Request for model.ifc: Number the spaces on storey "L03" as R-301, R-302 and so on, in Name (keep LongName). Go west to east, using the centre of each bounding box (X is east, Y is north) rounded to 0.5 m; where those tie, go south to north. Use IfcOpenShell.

First a look at what the model holds.

```python
import ifcopenshell
import ifcopenshell.util.element
import ifcopenshell.util.placement

model = ifcopenshell.open("model.ifc")
print(model.schema)
storey = next(s for s in model.by_type("IfcBuildingStorey") if s.Name == "L03")
spaces = [e for e in ifcopenshell.util.element.get_decomposition(storey) if e.is_a("IfcSpace")]
for e in sorted(spaces, key=lambda e: e.id()):
    origin = ifcopenshell.util.placement.get_local_placement(e.ObjectPlacement)[:3, 3]
    print(e.id(), e.Name, e.LongName, origin.round(2) + 0.0, sep=" | ")
```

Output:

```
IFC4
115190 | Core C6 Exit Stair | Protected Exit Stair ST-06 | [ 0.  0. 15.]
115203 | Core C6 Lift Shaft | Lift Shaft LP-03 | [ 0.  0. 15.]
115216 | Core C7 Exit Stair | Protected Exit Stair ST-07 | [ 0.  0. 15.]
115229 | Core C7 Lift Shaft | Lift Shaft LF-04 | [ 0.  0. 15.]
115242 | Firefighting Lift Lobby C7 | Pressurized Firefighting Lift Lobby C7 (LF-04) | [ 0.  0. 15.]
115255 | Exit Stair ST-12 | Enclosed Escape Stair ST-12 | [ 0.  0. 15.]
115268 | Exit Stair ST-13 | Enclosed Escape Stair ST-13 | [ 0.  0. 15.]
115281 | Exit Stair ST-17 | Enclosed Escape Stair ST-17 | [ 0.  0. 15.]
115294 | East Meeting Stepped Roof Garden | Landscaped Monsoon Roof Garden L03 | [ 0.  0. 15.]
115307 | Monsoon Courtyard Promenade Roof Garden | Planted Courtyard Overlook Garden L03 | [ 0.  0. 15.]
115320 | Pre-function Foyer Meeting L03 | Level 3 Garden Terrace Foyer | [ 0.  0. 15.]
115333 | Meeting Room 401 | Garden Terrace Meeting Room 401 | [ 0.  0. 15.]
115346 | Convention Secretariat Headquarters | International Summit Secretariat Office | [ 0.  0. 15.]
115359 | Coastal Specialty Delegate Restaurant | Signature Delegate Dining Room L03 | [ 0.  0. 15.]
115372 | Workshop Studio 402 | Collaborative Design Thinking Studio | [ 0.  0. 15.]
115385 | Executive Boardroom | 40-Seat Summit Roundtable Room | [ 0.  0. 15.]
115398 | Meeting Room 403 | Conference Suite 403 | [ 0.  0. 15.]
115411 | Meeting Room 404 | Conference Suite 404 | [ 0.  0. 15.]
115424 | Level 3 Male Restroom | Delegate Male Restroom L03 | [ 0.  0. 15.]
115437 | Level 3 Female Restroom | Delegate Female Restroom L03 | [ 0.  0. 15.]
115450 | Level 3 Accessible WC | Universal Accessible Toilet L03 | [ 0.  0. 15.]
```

```python
import ifcopenshell
import ifcopenshell.geom
import ifcopenshell.util.element
import ifcopenshell.util.shape

model = ifcopenshell.open("model.ifc")
settings = ifcopenshell.geom.settings()
settings.set("use-world-coords", True)


def centre(element):
    shape = ifcopenshell.geom.create_shape(settings, element)
    return ifcopenshell.util.shape.get_bbox_centroid(shape.geometry)


storey = next(s for s in model.by_type("IfcBuildingStorey") if s.Name == "L03")
spaces = [e for e in ifcopenshell.util.element.get_decomposition(storey) if e.is_a("IfcSpace")]

# Insertion points can sit at a corner or the storey origin, so sort by the geometry (in metres).
centres = {e: centre(e) for e in spaces}
spaces.sort(key=lambda e: (round(centres[e][0] / 0.5), centres[e][1]))

for i, e in enumerate(spaces, start=1):
    number = f"R-3{i:02d}"
    e.Name = number
    print(e.id(), number)

model.write("model_edited.ifc")
```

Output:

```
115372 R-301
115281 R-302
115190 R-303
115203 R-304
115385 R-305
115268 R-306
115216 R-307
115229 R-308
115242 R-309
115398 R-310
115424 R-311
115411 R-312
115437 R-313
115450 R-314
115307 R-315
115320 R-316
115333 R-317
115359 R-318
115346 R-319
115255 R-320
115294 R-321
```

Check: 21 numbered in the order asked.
